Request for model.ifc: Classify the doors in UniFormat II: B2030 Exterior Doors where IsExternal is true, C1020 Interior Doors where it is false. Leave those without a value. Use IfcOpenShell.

First a look at what the model holds.

```python
import ifcopenshell
import ifcopenshell.util.element

model = ifcopenshell.open("model.ifc")
print(model.schema)
print("classifications:", [c.Name for c in model.by_type("IfcClassification")])
values = [ifcopenshell.util.element.get_pset(e, "Pset_DoorCommon", "IsExternal") for e in model.by_type("IfcDoor")]
for value in (True, False, None):
    print("IsExternal", value, values.count(value))
```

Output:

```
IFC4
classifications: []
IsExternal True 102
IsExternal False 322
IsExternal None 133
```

```python
import ifcopenshell
import ifcopenshell.api.classification
import ifcopenshell.util.element

model = ifcopenshell.open("model.ifc")

system = ifcopenshell.api.classification.add_classification(model, classification="UniFormat II")

doors = model.by_type("IfcDoor")
external = {e: ifcopenshell.util.element.get_pset(e, "Pset_DoorCommon", "IsExternal") for e in doors}
for flag, code, name in ((True, "B2030", "Exterior Doors"), (False, "C1020", "Interior Doors")):
    products = [e for e in doors if external[e] is flag]
    ifcopenshell.api.classification.add_reference(
        model, products=products, classification=system, identification=code, name=name
    )
    print(code, len(products))

model.write("model_updated.ifc")
```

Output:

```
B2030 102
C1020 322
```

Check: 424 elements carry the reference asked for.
